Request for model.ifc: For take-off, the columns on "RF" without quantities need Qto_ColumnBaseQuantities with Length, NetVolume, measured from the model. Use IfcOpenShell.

First a look at what the model holds.

```python
import ifcopenshell
import ifcopenshell.util.element
import ifcopenshell.util.unit

model = ifcopenshell.open("model.ifc")
print(model.schema)
for unit_type in ("LENGTHUNIT", "AREAUNIT", "VOLUMEUNIT"):
    print(unit_type, ifcopenshell.util.unit.calculate_unit_scale(model, unit_type))
storey = next(s for s in model.by_type("IfcBuildingStorey") if s.Name == "RF")
columns = [e for e in ifcopenshell.util.element.get_decomposition(storey) if e.is_a("IfcColumn")]
for e in sorted(columns, key=lambda e: e.id()):
    print(e.id(), e.is_a(), e.Name, list(ifcopenshell.util.element.get_psets(e, qtos_only=True)), sep=" | ")
```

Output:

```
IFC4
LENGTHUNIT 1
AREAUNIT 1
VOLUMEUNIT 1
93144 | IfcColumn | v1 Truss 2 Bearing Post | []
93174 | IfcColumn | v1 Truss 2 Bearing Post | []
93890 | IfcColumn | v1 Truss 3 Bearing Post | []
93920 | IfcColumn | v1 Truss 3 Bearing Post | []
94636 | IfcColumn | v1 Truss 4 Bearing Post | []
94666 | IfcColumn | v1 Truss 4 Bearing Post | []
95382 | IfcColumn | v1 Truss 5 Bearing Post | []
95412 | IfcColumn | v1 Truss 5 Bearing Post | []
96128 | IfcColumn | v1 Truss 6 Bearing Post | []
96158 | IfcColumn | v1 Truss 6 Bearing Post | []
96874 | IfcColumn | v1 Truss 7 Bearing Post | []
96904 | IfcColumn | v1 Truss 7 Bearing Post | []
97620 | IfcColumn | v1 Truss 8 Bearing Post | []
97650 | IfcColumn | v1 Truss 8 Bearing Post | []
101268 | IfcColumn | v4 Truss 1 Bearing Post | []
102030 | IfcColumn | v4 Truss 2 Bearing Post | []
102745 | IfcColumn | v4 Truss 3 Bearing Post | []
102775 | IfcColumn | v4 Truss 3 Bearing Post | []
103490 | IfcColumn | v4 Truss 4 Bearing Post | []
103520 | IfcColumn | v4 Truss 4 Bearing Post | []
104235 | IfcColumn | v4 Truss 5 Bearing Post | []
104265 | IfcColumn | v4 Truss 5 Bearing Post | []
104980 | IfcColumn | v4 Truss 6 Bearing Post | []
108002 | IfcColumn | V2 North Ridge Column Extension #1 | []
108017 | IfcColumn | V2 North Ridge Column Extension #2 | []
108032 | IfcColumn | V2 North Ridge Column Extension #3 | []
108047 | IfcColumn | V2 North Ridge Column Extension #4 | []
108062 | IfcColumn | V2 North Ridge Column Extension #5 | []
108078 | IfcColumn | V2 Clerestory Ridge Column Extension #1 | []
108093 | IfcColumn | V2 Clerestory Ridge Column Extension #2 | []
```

```python
import ifcopenshell
import ifcopenshell.api.pset
import ifcopenshell.geom
import ifcopenshell.util.element
import ifcopenshell.util.shape
import ifcopenshell.util.unit

model = ifcopenshell.open("model.ifc")
unit_scale = ifcopenshell.util.unit.calculate_unit_scale(model)
volume_scale = ifcopenshell.util.unit.calculate_unit_scale(model, "VOLUMEUNIT")
settings = ifcopenshell.geom.settings()

storey = next(s for s in model.by_type("IfcBuildingStorey") if s.Name == "RF")
columns = [e for e in ifcopenshell.util.element.get_decomposition(storey) if e.is_a("IfcColumn")]

for e in sorted(columns, key=lambda e: e.id()):
    if ifcopenshell.util.element.get_psets(e, qtos_only=True, should_inherit=False):
        continue
    # Geometry comes back in metres, in the element's own axes.
    shape = ifcopenshell.geom.create_shape(settings, e)
    values = {
        "Length": ifcopenshell.util.shape.get_z(shape.geometry) / unit_scale,
        "NetVolume": ifcopenshell.util.shape.get_volume(shape.geometry) / volume_scale,
    }
    qto = ifcopenshell.api.pset.add_qto(model, product=e, name="Qto_ColumnBaseQuantities")
    ifcopenshell.api.pset.edit_qto(model, qto=qto, properties=values)
    print(e.id(), {k: round(v, 3) for k, v in values.items()})

model.write("model_v2.ifc")
```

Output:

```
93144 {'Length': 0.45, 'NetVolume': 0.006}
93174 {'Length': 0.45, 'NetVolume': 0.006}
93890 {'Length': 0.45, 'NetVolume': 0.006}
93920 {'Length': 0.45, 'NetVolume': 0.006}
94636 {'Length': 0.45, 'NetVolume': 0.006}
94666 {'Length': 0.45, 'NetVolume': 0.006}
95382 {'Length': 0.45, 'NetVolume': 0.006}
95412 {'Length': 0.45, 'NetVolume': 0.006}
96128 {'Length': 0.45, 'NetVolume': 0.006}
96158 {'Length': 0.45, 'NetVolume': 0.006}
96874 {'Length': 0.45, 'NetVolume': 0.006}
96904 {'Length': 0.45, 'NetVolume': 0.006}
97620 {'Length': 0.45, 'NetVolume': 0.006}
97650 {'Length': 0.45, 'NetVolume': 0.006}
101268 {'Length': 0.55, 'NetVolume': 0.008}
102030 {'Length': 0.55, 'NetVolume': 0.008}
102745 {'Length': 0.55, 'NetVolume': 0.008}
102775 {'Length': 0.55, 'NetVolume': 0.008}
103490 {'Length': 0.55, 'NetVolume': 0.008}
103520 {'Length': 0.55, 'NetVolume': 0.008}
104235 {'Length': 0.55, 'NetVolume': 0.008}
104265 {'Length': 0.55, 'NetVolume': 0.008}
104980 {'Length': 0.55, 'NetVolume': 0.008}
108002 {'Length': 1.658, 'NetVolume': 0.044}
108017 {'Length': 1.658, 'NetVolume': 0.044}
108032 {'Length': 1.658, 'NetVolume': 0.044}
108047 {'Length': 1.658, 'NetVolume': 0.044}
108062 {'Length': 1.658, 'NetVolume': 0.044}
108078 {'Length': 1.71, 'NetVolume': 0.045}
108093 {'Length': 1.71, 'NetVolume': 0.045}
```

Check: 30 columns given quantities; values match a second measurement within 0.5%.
